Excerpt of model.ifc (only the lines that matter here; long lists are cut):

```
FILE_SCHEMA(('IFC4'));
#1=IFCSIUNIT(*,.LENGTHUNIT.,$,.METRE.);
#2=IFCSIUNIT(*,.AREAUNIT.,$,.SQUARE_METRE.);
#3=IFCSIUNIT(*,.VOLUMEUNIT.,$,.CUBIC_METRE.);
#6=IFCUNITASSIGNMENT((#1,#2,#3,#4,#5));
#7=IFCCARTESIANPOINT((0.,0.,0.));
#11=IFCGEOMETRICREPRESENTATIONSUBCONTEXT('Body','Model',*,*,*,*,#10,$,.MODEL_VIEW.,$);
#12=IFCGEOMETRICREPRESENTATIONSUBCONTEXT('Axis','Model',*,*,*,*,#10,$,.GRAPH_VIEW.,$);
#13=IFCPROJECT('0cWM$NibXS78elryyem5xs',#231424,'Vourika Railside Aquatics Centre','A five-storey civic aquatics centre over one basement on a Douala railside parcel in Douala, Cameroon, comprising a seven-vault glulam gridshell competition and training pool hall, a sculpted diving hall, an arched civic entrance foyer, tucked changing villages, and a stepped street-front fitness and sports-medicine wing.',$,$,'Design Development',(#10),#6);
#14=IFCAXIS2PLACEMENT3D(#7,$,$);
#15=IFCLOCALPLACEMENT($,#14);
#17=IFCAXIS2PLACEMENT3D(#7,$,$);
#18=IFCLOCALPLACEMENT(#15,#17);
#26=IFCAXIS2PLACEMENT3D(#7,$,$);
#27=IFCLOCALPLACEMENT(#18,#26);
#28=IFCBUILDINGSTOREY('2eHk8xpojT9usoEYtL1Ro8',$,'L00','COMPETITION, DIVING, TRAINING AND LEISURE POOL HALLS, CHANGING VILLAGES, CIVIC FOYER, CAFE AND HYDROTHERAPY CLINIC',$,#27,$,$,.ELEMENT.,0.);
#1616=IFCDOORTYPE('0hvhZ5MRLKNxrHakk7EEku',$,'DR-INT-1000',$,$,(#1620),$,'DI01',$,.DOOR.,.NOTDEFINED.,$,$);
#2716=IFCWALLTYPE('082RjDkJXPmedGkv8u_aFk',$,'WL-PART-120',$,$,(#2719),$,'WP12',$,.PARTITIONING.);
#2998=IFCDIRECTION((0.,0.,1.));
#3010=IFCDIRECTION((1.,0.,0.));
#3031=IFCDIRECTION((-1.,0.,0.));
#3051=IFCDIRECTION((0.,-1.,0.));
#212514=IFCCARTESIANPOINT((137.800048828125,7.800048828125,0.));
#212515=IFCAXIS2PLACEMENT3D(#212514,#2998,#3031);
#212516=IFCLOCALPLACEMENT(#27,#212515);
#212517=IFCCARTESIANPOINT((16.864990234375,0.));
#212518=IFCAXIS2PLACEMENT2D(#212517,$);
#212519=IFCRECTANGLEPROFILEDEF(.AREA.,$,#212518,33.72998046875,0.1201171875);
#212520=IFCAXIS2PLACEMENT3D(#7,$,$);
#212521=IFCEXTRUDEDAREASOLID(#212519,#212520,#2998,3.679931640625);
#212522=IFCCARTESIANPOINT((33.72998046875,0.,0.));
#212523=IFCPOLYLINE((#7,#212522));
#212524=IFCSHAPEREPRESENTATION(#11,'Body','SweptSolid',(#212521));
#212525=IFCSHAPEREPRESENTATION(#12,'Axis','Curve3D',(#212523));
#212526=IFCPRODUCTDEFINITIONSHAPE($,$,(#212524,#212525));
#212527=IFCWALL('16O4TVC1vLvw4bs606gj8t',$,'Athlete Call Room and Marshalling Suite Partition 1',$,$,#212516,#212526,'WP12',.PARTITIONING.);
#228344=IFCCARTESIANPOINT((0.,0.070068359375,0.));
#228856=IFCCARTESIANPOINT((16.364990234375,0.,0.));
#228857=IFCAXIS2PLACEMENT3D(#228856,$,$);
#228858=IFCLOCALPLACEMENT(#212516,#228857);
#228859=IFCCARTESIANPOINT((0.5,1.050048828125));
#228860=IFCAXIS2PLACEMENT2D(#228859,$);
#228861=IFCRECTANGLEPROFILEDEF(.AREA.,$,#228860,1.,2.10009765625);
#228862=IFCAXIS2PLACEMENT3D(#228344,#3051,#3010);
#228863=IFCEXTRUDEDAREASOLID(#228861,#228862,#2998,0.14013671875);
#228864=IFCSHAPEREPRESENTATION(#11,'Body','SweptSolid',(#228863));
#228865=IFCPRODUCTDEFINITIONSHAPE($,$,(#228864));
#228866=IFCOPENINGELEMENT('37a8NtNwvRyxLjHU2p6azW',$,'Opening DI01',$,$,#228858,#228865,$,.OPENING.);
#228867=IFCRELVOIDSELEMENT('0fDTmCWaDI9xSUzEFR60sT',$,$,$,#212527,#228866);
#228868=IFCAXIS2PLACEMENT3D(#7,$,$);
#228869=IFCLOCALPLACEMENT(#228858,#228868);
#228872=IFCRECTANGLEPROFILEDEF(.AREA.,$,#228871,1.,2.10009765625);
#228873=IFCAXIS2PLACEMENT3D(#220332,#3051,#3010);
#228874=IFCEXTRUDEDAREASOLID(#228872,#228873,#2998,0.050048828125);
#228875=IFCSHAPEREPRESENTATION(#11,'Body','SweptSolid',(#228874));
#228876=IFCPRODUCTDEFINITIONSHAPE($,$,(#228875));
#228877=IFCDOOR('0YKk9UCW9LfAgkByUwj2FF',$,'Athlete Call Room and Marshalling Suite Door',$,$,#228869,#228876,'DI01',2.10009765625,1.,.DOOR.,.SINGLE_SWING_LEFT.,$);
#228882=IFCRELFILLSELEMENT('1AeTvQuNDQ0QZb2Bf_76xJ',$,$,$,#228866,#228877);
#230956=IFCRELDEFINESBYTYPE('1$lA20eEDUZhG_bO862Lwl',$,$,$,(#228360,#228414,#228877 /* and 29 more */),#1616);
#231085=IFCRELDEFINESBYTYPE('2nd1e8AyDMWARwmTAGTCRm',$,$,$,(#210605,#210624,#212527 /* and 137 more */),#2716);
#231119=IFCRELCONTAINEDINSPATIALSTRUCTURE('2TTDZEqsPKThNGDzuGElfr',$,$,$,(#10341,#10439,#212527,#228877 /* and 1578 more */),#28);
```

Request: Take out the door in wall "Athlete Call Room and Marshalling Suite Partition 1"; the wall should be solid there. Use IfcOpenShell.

```python
import ifcopenshell
import ifcopenshell.api.feature
import ifcopenshell.api.root
import ifcopenshell.geom
import ifcopenshell.util.shape

model = ifcopenshell.open("model.ifc")
settings = ifcopenshell.geom.settings()


def volume(element):
    """Net volume in cubic metres, openings subtracted."""
    shape = ifcopenshell.geom.create_shape(settings, element)
    return ifcopenshell.util.shape.get_volume(shape.geometry)


door = model.by_id(228877)
opening = door.FillsVoids[0].RelatingOpeningElement
wall = opening.VoidsElements[0].RelatingBuildingElement
before = volume(wall)

ifcopenshell.api.root.remove_product(model, product=door)
ifcopenshell.api.feature.remove_feature(model, feature=opening)

after = volume(wall)

print(f"wall volume {before:.3f} -> {after:.3f} m3")

model.write("model_rev.ifc")
```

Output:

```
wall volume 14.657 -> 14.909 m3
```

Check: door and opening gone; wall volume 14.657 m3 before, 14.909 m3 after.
